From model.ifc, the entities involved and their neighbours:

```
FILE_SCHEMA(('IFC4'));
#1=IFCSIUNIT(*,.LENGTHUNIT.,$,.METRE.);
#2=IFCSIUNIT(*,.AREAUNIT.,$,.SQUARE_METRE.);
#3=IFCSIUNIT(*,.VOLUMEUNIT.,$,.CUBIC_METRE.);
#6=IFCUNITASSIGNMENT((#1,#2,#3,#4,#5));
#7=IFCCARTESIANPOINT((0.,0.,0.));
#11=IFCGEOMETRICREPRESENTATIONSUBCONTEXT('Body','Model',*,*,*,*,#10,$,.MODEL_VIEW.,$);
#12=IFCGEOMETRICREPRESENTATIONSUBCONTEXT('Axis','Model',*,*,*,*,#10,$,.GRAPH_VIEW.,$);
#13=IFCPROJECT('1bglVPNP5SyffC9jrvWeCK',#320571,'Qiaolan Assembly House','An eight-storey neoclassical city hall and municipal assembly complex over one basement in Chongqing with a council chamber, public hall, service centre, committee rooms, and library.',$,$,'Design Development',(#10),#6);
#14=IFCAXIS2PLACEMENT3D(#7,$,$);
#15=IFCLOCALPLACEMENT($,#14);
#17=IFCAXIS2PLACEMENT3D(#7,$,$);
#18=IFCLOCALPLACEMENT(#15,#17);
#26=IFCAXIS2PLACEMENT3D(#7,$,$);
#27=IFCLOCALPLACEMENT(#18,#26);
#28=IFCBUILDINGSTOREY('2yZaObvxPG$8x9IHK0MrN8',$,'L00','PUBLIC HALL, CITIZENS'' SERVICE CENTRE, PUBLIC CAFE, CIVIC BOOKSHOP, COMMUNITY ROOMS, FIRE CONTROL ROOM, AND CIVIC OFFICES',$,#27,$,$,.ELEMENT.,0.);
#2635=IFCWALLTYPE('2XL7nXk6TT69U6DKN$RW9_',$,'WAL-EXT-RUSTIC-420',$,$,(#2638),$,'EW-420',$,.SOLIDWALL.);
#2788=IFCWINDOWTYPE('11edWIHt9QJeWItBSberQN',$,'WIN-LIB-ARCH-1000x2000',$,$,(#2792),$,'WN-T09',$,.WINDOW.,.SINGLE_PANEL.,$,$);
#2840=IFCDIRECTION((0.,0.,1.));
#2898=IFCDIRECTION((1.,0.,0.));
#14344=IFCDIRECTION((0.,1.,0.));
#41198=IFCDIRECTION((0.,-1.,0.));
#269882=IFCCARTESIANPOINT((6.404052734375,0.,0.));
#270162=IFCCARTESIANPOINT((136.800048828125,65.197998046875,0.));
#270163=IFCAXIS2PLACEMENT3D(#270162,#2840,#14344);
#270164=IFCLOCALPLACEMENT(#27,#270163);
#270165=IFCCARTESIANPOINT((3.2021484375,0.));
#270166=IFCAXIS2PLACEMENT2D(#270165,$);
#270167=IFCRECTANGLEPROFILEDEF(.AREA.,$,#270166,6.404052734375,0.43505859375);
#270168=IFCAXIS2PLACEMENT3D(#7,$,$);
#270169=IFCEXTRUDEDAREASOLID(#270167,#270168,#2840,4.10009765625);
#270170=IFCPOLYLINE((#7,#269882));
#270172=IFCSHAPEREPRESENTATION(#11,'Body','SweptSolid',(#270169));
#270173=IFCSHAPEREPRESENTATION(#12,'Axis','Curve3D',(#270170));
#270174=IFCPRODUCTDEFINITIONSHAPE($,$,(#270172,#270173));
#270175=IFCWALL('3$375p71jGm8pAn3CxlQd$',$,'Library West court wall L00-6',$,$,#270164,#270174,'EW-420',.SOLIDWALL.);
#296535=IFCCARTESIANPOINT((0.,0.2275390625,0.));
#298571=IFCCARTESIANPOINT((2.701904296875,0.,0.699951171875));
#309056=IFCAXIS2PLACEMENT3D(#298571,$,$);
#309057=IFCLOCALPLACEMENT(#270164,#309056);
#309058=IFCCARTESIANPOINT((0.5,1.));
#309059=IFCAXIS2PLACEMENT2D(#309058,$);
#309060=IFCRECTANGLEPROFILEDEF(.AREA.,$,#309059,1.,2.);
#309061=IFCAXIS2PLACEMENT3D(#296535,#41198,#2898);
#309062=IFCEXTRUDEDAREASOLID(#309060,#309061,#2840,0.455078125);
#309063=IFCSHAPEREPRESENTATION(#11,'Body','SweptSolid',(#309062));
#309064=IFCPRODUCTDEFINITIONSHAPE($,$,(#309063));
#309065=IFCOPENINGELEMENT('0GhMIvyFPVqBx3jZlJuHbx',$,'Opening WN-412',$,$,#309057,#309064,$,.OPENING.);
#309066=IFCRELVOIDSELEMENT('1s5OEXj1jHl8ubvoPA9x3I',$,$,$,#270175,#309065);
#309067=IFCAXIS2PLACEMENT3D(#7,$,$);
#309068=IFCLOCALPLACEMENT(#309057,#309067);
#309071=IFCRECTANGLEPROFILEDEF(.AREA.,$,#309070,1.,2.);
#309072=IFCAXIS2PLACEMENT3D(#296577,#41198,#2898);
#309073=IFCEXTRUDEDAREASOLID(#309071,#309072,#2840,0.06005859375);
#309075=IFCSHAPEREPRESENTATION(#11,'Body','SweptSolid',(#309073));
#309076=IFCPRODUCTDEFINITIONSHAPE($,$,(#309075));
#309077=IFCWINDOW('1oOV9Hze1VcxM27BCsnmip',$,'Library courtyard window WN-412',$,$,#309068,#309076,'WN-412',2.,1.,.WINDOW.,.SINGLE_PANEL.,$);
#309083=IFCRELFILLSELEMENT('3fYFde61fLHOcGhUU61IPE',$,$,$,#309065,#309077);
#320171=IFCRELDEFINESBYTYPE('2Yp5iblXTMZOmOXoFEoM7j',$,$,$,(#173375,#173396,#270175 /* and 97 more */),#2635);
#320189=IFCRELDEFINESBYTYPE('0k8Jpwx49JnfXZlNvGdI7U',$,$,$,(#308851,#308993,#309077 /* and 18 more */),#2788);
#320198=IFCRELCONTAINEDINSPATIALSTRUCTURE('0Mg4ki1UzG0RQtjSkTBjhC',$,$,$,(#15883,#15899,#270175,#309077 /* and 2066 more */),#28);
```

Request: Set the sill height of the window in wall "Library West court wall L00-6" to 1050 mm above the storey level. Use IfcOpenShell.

```python
import numpy as np
import ifcopenshell
import ifcopenshell.api.geometry
import ifcopenshell.geom
import ifcopenshell.util.element
import ifcopenshell.util.placement
import ifcopenshell.util.shape
import ifcopenshell.util.unit

model = ifcopenshell.open("model.ifc")
unit_scale = ifcopenshell.util.unit.calculate_unit_scale(model)

window = model.by_guid("1oOV9Hze1VcxM27BCsnmip")
opening = window.FillsVoids[0].RelatingOpeningElement
storey = ifcopenshell.util.element.get_container(window, ifc_class="IfcBuildingStorey")
level = ifcopenshell.util.placement.get_local_placement(storey.ObjectPlacement)[2, 3]

# The opening's origin need not be at the sill, so measure its lowest point.
shape = ifcopenshell.geom.create_shape(ifcopenshell.geom.settings(), opening)
bottom = ifcopenshell.util.shape.get_shape_bottom_elevation(shape, shape.geometry) / unit_scale
dz = level + 1.05 / unit_scale - bottom

shift = np.array([0.0, 0.0, dz])
# The window is placed relative to its opening, so it follows when the opening moves.
matrix = ifcopenshell.util.placement.get_local_placement(opening.ObjectPlacement)
matrix[:3, 3] += shift
ifcopenshell.api.geometry.edit_object_placement(
    model, product=opening, matrix=matrix, is_si=False, should_transform_children=True
)

print(f"moved by {dz * unit_scale:+.3f} m")

model.write("model_v2.ifc")
```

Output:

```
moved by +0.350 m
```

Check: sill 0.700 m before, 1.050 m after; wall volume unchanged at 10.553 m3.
